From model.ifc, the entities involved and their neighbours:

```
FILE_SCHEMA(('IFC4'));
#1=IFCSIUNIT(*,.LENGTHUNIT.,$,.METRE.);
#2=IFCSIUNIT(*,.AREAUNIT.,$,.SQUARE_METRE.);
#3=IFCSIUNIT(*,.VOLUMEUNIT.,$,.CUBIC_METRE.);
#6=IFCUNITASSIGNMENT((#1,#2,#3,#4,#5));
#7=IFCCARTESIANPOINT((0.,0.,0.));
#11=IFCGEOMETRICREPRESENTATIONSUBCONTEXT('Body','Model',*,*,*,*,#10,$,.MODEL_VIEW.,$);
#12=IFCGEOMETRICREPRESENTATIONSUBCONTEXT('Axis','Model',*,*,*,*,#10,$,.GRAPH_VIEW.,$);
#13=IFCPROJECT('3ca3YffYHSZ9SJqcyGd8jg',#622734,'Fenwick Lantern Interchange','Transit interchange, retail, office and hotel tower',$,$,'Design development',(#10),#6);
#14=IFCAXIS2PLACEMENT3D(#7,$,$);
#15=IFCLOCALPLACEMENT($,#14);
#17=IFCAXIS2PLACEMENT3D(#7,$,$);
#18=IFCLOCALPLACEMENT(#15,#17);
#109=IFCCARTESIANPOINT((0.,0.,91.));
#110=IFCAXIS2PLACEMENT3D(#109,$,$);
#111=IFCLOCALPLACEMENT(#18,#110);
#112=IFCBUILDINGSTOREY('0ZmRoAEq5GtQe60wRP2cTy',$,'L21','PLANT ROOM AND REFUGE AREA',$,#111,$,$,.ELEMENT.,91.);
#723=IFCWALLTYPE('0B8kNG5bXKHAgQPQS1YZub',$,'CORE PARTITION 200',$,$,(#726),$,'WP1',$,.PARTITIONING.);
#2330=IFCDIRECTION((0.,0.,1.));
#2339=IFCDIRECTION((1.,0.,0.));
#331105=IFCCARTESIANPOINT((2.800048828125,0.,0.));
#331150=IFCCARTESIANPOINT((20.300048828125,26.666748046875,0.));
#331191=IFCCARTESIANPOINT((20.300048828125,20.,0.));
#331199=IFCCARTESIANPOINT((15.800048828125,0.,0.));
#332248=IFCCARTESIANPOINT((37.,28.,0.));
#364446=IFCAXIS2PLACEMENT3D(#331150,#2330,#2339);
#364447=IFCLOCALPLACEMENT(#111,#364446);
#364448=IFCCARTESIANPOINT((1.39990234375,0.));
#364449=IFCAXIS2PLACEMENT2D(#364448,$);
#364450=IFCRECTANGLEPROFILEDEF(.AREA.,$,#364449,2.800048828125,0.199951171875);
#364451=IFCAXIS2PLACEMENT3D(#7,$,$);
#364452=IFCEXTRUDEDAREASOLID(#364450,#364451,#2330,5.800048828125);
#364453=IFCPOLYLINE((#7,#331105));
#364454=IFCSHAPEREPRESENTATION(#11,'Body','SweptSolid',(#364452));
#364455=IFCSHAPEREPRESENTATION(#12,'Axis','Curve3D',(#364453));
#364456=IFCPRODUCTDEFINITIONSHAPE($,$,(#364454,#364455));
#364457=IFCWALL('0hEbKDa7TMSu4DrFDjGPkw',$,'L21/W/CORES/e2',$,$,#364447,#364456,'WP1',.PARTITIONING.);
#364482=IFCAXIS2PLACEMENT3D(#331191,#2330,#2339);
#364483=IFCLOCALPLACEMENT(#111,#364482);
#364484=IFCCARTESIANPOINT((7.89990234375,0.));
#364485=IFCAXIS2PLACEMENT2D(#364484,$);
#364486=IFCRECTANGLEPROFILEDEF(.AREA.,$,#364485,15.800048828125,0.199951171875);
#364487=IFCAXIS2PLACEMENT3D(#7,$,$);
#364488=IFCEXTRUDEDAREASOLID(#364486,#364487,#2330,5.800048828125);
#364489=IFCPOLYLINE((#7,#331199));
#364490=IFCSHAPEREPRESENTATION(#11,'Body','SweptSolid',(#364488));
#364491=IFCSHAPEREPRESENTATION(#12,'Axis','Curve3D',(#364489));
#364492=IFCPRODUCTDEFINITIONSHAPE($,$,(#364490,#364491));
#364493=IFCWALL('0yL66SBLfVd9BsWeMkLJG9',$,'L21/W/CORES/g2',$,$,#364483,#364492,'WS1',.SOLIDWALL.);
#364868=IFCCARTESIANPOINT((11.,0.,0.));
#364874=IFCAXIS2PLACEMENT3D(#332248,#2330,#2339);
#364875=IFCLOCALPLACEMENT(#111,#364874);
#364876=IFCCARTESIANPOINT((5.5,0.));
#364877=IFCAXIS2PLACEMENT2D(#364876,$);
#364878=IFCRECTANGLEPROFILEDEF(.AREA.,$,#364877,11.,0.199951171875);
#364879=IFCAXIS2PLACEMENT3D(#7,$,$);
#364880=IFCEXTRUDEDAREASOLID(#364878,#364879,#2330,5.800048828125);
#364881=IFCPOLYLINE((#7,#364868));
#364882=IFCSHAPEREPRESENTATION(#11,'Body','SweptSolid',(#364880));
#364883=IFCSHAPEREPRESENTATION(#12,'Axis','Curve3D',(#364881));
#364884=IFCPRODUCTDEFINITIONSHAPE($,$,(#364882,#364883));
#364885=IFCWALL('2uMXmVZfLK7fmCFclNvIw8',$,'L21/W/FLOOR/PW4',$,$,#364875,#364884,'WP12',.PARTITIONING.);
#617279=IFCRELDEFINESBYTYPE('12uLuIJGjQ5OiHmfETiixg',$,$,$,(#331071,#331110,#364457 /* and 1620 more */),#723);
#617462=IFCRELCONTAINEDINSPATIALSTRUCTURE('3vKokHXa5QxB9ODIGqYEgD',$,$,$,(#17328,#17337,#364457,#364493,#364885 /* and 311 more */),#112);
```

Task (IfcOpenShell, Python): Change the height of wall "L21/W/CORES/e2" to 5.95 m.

```python
import ifcopenshell
import ifcopenshell.geom
import ifcopenshell.util.representation
import ifcopenshell.util.shape
import ifcopenshell.util.unit

model = ifcopenshell.open("model.ifc")
unit_scale = ifcopenshell.util.unit.calculate_unit_scale(model)
settings = ifcopenshell.geom.settings()


def volume(element):
    """Net volume in cubic metres, openings subtracted."""
    shape = ifcopenshell.geom.create_shape(settings, element)
    return ifcopenshell.util.shape.get_volume(shape.geometry)


wall = model.by_guid("0hEbKDa7TMSu4DrFDjGPkw")
before = volume(wall)

body = ifcopenshell.util.representation.get_representation(wall, "Model", "Body")
solid = body.Items[0]
old_height = solid.Depth
solid.Depth = 5.95 / unit_scale
after = volume(wall)

print(f"height {old_height:g} -> {solid.Depth:g}, volume {before:.3f} -> {after:.3f} m3")

model.write("model_edited.ifc")
```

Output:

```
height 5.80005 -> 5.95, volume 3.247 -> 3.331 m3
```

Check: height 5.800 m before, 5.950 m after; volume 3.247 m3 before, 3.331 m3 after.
